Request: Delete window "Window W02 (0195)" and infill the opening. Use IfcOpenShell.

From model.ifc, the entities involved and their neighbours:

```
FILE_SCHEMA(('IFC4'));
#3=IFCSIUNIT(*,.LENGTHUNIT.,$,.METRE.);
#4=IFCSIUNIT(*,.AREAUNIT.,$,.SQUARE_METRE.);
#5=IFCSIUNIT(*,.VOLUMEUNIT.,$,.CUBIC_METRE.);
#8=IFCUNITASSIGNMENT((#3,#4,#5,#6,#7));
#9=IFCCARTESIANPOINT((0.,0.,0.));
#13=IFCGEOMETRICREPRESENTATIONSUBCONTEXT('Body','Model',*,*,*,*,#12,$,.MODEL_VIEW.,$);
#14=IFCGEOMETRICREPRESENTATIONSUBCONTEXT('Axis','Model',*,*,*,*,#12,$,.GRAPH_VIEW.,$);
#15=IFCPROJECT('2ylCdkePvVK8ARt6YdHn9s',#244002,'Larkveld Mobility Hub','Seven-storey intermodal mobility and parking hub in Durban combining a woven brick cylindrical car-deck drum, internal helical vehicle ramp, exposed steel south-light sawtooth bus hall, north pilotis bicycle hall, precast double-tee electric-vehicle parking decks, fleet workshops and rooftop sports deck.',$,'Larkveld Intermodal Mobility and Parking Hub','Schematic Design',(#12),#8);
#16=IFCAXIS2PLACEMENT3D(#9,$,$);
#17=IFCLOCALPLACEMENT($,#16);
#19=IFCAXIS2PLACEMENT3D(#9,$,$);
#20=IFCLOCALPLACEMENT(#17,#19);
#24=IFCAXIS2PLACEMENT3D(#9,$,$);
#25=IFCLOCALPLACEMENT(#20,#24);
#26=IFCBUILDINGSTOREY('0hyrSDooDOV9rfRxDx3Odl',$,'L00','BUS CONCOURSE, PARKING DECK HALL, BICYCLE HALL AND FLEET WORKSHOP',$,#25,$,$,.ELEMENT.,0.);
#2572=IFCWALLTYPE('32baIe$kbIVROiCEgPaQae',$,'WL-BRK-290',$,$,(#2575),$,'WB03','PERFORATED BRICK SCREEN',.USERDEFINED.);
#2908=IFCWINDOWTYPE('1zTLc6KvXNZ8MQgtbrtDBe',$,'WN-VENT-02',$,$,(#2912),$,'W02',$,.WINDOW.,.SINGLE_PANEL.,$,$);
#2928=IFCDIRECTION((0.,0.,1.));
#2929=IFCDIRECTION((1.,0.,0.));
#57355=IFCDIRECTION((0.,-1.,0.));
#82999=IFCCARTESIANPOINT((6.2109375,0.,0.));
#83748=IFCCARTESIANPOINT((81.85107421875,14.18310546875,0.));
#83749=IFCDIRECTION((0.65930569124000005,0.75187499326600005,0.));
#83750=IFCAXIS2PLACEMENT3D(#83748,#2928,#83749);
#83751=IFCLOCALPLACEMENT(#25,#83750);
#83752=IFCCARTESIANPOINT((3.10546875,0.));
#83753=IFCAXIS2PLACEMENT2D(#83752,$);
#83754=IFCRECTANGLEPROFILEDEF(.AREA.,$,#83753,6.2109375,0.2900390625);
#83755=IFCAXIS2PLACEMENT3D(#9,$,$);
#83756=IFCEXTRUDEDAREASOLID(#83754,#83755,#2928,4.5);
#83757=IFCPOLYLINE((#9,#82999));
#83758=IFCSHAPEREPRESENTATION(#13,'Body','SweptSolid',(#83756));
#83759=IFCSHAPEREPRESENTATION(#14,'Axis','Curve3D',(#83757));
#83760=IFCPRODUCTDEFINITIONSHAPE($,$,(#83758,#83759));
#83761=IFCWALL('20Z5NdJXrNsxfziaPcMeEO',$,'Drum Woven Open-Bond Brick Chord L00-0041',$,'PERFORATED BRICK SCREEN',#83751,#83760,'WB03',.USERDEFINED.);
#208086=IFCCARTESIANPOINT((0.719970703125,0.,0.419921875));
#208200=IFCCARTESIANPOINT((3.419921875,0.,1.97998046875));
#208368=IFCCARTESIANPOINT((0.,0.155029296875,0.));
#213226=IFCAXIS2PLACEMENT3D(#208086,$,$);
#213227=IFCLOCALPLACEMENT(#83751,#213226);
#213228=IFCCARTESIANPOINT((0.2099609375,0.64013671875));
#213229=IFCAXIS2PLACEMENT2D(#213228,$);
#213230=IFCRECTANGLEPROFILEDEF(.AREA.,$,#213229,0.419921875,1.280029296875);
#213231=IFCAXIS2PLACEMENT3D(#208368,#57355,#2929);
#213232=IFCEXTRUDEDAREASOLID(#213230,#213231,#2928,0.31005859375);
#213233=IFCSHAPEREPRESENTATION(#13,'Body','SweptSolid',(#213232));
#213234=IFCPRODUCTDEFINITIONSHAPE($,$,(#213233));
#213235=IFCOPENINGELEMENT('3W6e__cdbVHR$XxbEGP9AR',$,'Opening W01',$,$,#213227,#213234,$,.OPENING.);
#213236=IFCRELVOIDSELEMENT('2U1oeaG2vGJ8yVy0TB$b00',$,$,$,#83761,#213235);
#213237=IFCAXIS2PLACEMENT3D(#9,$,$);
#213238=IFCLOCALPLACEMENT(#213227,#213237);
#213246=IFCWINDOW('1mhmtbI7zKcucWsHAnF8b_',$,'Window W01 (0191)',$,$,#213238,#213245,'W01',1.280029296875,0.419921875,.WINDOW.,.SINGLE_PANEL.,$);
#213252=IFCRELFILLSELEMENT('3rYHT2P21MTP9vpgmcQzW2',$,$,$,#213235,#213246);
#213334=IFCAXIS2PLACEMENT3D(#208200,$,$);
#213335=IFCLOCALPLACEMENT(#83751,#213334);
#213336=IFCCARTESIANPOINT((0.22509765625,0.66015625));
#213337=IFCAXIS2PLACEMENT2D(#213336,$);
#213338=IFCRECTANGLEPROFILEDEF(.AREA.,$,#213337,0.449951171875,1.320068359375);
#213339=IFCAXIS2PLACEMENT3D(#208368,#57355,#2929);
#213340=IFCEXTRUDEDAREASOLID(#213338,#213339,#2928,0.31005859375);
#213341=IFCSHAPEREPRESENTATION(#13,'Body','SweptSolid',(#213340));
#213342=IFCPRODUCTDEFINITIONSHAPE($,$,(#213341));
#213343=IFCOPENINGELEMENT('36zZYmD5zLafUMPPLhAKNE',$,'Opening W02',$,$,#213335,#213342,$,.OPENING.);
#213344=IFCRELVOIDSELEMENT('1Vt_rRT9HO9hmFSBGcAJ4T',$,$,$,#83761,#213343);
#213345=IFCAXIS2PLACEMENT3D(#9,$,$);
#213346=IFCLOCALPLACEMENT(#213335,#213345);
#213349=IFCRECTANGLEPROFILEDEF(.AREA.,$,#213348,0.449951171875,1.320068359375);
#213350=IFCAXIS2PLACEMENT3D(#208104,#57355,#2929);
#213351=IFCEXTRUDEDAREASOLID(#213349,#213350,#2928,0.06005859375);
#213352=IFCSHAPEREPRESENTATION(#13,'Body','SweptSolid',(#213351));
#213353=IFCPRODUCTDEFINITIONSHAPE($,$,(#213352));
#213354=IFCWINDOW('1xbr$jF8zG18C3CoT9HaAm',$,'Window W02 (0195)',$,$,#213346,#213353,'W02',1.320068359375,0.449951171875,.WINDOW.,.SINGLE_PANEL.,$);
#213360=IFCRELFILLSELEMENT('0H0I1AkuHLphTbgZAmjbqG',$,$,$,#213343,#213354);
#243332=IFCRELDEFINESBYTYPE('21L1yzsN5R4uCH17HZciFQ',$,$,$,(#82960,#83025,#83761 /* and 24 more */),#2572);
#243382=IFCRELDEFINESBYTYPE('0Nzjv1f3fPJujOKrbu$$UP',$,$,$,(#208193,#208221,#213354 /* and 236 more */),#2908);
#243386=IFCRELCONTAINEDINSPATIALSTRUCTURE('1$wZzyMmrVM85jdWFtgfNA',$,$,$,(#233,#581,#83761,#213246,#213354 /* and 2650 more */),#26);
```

```python
import ifcopenshell
import ifcopenshell.api.feature
import ifcopenshell.api.root
import ifcopenshell.geom
import ifcopenshell.util.shape

model = ifcopenshell.open("model.ifc")
settings = ifcopenshell.geom.settings()


def volume(element):
    """Net volume in cubic metres, openings subtracted."""
    shape = ifcopenshell.geom.create_shape(settings, element)
    return ifcopenshell.util.shape.get_volume(shape.geometry)


window = model.by_id(213354)
opening = window.FillsVoids[0].RelatingOpeningElement
wall = opening.VoidsElements[0].RelatingBuildingElement
before = volume(wall)

ifcopenshell.api.root.remove_product(model, product=window)
ifcopenshell.api.feature.remove_feature(model, feature=opening)

after = volume(wall)

print(f"wall volume {before:.3f} -> {after:.3f} m3")

model.write("model_rev.ifc")
```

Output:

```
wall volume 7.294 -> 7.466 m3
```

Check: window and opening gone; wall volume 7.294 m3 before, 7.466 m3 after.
